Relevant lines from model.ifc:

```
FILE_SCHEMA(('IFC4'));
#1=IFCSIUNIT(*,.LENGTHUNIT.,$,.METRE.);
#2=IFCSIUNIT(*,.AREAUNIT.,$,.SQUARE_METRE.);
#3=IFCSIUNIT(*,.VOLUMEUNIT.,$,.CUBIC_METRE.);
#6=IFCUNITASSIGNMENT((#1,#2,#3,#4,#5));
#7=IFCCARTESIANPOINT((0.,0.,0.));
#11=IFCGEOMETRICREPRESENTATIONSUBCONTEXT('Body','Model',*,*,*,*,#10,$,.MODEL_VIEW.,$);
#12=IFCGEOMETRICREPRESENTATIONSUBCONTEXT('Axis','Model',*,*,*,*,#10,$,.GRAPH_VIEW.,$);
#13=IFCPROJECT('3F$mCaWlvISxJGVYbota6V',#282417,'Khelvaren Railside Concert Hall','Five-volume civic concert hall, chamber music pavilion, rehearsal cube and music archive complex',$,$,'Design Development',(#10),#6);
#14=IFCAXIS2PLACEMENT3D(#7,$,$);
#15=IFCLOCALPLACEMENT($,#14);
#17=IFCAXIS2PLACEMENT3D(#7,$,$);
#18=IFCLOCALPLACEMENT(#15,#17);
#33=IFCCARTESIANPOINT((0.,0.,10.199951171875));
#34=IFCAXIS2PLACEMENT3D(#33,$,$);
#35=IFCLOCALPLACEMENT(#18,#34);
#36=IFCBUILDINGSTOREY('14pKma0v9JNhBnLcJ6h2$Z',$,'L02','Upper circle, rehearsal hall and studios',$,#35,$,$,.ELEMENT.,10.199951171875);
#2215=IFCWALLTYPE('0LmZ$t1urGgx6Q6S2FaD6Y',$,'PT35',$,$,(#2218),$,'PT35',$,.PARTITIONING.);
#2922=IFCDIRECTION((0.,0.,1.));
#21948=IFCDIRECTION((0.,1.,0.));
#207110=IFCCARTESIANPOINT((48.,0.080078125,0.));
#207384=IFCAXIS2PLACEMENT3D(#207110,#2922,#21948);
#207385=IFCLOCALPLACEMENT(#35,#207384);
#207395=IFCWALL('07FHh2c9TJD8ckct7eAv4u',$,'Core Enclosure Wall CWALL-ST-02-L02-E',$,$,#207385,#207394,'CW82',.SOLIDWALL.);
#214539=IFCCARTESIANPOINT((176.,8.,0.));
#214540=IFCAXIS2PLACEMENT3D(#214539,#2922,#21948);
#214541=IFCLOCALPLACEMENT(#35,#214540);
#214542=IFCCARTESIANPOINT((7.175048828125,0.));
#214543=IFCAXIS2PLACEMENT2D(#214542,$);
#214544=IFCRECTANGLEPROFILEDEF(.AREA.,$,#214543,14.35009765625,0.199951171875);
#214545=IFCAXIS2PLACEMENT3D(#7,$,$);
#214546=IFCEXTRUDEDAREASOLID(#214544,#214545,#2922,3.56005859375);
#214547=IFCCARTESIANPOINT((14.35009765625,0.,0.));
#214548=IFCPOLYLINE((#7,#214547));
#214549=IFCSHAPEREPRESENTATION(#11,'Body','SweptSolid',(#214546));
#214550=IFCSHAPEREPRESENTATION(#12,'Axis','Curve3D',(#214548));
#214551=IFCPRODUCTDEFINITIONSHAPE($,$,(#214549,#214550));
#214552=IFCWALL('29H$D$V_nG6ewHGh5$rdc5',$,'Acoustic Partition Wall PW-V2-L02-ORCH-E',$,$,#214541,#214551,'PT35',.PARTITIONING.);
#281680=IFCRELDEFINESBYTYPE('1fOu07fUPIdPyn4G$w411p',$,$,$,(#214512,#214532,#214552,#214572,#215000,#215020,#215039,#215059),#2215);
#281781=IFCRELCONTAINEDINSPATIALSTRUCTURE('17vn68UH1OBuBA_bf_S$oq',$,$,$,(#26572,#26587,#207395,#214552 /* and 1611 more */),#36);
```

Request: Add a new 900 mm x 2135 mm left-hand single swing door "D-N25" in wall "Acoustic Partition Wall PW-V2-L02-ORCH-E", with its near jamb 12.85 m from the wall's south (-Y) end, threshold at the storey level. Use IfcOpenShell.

```python
import numpy as np
import ifcopenshell
import ifcopenshell.api.feature
import ifcopenshell.api.geometry
import ifcopenshell.api.root
import ifcopenshell.api.spatial
import ifcopenshell.geom
import ifcopenshell.util.element
import ifcopenshell.util.placement
import ifcopenshell.util.representation
import ifcopenshell.util.shape
import ifcopenshell.util.unit

model = ifcopenshell.open("model.ifc")
unit_scale = ifcopenshell.util.unit.calculate_unit_scale(model)
settings = ifcopenshell.geom.settings()


def volume(element):
    """Net volume in cubic metres, openings subtracted."""
    shape = ifcopenshell.geom.create_shape(settings, element)
    return ifcopenshell.util.shape.get_volume(shape.geometry)


wall = model.by_guid("29H$D$V_nG6ewHGh5$rdc5")
storey = ifcopenshell.util.element.get_container(wall, ifc_class="IfcBuildingStorey")
context = ifcopenshell.util.representation.get_context(model, "Model", "Body", "MODEL_VIEW")
before = volume(wall)

width, height, from_end, sill = 0.9, 2.135, 12.85, 0.0  # metres

# The wall runs along its own X axis, and the end named is its -X end.
wall_shape = ifcopenshell.geom.create_shape(settings, wall)
x, y, z = ifcopenshell.util.shape.get_vertices(wall_shape.geometry).T
start = x.min() + from_end
face, thickness = float(y.min()), float(y.max() - y.min())
wall_matrix = ifcopenshell.util.placement.get_local_placement(wall.ObjectPlacement)
level = ifcopenshell.util.placement.get_local_placement(storey.ObjectPlacement)[2, 3]


def in_wall(x, y):
    """Placement at x, y metres in the wall's axes, at sill height."""
    matrix = wall_matrix.copy()
    matrix[:, 3] = wall_matrix @ np.array([x / unit_scale, y / unit_scale, 0.0, 1.0])
    matrix[2, 3] = level + sill / unit_scale
    return matrix


# Opening: a box that overshoots both wall faces by 50 mm.
opening = ifcopenshell.api.root.create_entity(model, ifc_class="IfcOpeningElement", predefined_type="OPENING")
box = ifcopenshell.api.geometry.add_wall_representation(
    model, context=context, length=width, height=height, thickness=thickness + 0.1
)
ifcopenshell.api.geometry.assign_representation(model, product=opening, representation=box)
ifcopenshell.api.geometry.edit_object_placement(model, product=opening, matrix=in_wall(start, face - 0.05), is_si=False)
ifcopenshell.api.feature.add_feature(model, feature=opening, element=wall)

door = ifcopenshell.api.root.create_entity(model, ifc_class="IfcDoor", name="D-N25", predefined_type="DOOR")
door.OverallWidth, door.OverallHeight = width / unit_scale, height / unit_scale
door.OperationType = "SINGLE_SWING_LEFT"
body = ifcopenshell.api.geometry.add_door_representation(
    model,
    context=context,
    overall_width=door.OverallWidth,
    overall_height=door.OverallHeight,
    operation_type="SINGLE_SWING_LEFT",
    lining_properties={"LiningDepth": thickness / unit_scale, "ThresholdDepth": thickness / unit_scale},
)
ifcopenshell.api.geometry.assign_representation(model, product=door, representation=body)
ifcopenshell.api.spatial.assign_container(model, products=[door], relating_structure=storey)
ifcopenshell.api.feature.add_filling(model, opening=opening, element=door)

# The lining spans the wall, so the door starts at the wall face.
ifcopenshell.api.geometry.edit_object_placement(model, product=door, matrix=in_wall(start, face), is_si=False)

after = volume(wall)

print(f"wall volume {before:.3f} -> {after:.3f} m3")

model.write("model_rev.ifc")
```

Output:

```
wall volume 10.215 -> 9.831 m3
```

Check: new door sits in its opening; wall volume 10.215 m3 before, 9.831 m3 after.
